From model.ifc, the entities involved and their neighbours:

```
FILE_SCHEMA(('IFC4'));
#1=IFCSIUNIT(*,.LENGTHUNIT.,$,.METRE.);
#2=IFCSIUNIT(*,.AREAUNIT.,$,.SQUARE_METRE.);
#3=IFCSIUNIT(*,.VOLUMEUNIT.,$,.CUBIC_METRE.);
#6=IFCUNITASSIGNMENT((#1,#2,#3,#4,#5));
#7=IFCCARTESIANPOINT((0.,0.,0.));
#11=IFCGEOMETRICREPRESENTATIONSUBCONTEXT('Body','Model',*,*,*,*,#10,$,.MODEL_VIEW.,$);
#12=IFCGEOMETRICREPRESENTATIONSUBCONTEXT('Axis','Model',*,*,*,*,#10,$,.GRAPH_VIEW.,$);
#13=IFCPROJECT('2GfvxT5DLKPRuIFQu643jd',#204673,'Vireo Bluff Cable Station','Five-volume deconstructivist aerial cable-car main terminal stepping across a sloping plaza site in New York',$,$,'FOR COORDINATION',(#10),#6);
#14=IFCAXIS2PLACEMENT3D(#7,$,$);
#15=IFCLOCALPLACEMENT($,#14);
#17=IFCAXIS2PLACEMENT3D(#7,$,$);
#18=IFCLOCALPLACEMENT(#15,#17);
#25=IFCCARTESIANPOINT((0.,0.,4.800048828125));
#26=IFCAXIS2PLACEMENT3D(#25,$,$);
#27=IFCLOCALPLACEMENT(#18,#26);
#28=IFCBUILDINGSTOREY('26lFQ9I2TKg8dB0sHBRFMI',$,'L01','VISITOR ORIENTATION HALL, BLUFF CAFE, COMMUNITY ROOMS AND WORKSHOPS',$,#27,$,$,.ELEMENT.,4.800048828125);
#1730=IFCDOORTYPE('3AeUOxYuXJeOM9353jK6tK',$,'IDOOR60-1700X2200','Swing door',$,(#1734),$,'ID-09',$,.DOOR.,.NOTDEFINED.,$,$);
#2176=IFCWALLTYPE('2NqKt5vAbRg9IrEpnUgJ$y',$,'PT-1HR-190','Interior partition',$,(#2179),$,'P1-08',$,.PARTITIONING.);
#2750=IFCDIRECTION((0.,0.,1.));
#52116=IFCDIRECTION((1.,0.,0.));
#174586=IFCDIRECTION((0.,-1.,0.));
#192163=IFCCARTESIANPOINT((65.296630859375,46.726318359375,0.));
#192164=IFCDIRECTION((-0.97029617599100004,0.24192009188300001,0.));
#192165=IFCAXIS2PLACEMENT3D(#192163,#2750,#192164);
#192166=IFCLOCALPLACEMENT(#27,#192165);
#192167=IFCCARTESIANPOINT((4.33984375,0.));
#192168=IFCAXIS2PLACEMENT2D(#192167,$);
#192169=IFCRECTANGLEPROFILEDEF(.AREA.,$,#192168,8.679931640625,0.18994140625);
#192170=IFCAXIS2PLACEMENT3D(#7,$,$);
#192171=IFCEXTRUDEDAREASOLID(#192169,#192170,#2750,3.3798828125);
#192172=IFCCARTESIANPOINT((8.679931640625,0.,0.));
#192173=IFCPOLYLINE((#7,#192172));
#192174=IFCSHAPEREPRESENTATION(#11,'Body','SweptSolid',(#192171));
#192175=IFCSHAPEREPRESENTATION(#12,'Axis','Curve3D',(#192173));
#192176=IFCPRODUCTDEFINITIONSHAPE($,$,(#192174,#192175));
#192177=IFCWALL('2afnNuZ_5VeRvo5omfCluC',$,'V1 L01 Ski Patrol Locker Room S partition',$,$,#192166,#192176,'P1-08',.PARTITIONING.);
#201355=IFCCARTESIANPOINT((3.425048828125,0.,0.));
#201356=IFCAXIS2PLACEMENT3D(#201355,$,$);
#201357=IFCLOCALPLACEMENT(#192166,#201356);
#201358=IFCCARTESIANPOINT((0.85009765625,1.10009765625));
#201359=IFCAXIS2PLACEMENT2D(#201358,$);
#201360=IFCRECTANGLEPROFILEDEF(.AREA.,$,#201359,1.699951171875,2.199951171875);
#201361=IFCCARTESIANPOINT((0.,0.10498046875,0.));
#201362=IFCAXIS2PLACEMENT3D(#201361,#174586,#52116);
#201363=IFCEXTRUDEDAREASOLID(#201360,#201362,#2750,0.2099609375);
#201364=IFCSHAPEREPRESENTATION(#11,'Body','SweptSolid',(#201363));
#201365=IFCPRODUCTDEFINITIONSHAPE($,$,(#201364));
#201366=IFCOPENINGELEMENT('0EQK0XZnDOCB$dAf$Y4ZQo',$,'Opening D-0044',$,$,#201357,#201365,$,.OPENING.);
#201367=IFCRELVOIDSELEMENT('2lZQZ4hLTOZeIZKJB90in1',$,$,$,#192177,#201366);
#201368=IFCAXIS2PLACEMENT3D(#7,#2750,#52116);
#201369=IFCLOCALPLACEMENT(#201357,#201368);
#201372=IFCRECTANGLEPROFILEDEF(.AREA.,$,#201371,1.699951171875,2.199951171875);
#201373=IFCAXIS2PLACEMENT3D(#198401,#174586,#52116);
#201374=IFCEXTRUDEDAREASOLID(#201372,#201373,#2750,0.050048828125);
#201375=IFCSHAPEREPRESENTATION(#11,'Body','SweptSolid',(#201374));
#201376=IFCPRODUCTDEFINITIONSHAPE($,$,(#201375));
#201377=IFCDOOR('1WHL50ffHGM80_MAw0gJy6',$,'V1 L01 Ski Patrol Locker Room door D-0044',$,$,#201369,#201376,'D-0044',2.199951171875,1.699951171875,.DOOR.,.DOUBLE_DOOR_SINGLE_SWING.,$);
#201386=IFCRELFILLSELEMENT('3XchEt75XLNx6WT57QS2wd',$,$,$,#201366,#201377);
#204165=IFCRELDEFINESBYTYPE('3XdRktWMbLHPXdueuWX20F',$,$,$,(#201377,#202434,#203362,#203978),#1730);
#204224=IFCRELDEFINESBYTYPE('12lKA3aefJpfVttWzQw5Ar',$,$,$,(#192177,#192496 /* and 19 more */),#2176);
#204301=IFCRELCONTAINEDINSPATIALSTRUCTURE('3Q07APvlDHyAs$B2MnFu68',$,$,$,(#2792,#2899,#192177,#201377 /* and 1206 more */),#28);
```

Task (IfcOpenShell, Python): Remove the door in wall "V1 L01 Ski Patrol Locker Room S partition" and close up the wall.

```python
import ifcopenshell
import ifcopenshell.api.feature
import ifcopenshell.api.root
import ifcopenshell.geom
import ifcopenshell.util.shape

model = ifcopenshell.open("model.ifc")
settings = ifcopenshell.geom.settings()


def volume(element):
    """Net volume in cubic metres, openings subtracted."""
    shape = ifcopenshell.geom.create_shape(settings, element)
    return ifcopenshell.util.shape.get_volume(shape.geometry)


door = model.by_id(201377)
opening = door.FillsVoids[0].RelatingOpeningElement
wall = opening.VoidsElements[0].RelatingBuildingElement
before = volume(wall)

ifcopenshell.api.root.remove_product(model, product=door)
ifcopenshell.api.feature.remove_feature(model, feature=opening)

after = volume(wall)

print(f"wall volume {before:.3f} -> {after:.3f} m3")

model.write("model_rev.ifc")
```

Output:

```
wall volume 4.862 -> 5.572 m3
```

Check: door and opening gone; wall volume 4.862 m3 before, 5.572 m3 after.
